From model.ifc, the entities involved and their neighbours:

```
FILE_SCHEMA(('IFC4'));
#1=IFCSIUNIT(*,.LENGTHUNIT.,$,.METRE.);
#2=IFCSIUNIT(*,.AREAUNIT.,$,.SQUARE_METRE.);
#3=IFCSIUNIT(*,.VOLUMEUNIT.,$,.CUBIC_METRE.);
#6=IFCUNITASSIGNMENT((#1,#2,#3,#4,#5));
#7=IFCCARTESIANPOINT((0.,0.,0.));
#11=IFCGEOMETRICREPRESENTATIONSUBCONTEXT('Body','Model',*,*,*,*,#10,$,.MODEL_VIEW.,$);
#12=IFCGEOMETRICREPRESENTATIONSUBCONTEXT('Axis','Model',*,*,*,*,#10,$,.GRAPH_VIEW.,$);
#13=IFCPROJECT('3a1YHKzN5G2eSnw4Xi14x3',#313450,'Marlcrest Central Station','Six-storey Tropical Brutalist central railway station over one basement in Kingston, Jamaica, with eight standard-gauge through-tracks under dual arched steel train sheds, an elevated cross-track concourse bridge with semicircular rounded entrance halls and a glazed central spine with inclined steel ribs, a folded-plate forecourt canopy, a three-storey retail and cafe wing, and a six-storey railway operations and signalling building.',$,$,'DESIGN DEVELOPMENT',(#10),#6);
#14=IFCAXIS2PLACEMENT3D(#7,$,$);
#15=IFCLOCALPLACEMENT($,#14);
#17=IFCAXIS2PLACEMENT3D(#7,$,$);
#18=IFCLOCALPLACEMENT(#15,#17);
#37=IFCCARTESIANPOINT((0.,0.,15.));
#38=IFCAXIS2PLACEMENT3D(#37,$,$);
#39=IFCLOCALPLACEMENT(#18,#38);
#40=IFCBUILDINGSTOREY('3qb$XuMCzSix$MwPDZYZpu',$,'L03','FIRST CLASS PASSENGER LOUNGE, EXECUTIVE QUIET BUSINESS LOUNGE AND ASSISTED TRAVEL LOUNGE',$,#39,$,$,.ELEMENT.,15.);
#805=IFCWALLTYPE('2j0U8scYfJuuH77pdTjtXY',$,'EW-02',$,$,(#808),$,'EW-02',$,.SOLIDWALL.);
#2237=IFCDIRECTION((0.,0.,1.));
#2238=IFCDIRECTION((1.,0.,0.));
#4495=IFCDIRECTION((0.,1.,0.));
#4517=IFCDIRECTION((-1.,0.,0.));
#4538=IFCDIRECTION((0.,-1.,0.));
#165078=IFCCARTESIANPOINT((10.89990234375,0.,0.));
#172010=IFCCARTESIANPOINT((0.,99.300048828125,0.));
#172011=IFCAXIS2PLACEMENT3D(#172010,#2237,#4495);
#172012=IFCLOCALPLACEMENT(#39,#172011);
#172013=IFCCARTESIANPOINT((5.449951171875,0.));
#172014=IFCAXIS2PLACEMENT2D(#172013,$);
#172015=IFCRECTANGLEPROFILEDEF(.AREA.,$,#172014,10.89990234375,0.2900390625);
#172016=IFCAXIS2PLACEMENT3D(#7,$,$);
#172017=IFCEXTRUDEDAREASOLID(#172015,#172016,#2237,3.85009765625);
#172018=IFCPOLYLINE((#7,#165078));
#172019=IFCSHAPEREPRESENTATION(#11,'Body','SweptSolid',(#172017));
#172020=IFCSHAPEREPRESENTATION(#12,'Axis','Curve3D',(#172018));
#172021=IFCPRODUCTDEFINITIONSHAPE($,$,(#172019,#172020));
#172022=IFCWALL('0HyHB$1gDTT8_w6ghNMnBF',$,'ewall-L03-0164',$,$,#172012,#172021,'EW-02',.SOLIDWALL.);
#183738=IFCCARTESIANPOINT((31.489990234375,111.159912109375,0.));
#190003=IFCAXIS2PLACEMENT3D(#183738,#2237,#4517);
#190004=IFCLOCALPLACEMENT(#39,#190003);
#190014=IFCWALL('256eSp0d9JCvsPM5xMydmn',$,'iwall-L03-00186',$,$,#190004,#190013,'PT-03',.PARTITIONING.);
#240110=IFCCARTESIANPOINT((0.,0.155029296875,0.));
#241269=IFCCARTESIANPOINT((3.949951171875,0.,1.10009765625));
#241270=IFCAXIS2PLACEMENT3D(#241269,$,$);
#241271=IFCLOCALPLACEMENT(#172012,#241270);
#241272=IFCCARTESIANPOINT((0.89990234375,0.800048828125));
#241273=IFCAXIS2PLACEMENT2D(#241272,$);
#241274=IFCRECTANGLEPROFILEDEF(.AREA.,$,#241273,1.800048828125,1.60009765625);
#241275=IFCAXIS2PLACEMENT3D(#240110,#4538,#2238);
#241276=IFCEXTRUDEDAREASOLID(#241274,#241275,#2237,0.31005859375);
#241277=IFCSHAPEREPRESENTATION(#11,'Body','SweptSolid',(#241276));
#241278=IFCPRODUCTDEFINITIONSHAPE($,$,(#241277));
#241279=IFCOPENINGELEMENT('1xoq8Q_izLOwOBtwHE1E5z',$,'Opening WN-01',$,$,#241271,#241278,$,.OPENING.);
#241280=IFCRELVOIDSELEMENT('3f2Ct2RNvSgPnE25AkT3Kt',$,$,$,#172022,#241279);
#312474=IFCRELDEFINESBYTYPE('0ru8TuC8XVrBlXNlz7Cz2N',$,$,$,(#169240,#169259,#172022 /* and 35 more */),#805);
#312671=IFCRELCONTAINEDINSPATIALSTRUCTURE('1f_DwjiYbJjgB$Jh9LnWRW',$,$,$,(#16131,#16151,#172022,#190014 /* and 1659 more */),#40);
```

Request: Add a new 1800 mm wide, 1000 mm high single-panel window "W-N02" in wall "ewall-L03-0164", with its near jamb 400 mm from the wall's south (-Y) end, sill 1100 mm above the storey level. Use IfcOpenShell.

```python
import numpy as np
import ifcopenshell
import ifcopenshell.api.feature
import ifcopenshell.api.geometry
import ifcopenshell.api.root
import ifcopenshell.api.spatial
import ifcopenshell.geom
import ifcopenshell.util.element
import ifcopenshell.util.placement
import ifcopenshell.util.representation
import ifcopenshell.util.shape
import ifcopenshell.util.unit

model = ifcopenshell.open("model.ifc")
unit_scale = ifcopenshell.util.unit.calculate_unit_scale(model)
settings = ifcopenshell.geom.settings()


def volume(element):
    """Net volume in cubic metres, openings subtracted."""
    shape = ifcopenshell.geom.create_shape(settings, element)
    return ifcopenshell.util.shape.get_volume(shape.geometry)


wall = model.by_guid("0HyHB$1gDTT8_w6ghNMnBF")
storey = ifcopenshell.util.element.get_container(wall, ifc_class="IfcBuildingStorey")
context = ifcopenshell.util.representation.get_context(model, "Model", "Body", "MODEL_VIEW")
before = volume(wall)

width, height, from_end, sill = 1.8, 1, 0.4, 1.1  # metres

# The wall runs along its own X axis, and the end named is its -X end.
wall_shape = ifcopenshell.geom.create_shape(settings, wall)
x, y, z = ifcopenshell.util.shape.get_vertices(wall_shape.geometry).T
start = x.min() + from_end
face, thickness = float(y.min()), float(y.max() - y.min())
wall_matrix = ifcopenshell.util.placement.get_local_placement(wall.ObjectPlacement)
level = ifcopenshell.util.placement.get_local_placement(storey.ObjectPlacement)[2, 3]


def in_wall(x, y):
    """Placement at x, y metres in the wall's axes, at sill height."""
    matrix = wall_matrix.copy()
    matrix[:, 3] = wall_matrix @ np.array([x / unit_scale, y / unit_scale, 0.0, 1.0])
    matrix[2, 3] = level + sill / unit_scale
    return matrix


# Opening: a box that overshoots both wall faces by 50 mm.
opening = ifcopenshell.api.root.create_entity(model, ifc_class="IfcOpeningElement", predefined_type="OPENING")
box = ifcopenshell.api.geometry.add_wall_representation(
    model, context=context, length=width, height=height, thickness=thickness + 0.1
)
ifcopenshell.api.geometry.assign_representation(model, product=opening, representation=box)
ifcopenshell.api.geometry.edit_object_placement(model, product=opening, matrix=in_wall(start, face - 0.05), is_si=False)
ifcopenshell.api.feature.add_feature(model, feature=opening, element=wall)

window = ifcopenshell.api.root.create_entity(model, ifc_class="IfcWindow", name="W-N02", predefined_type="WINDOW")
window.OverallWidth, window.OverallHeight = width / unit_scale, height / unit_scale
window.PartitioningType = "SINGLE_PANEL"
body = ifcopenshell.api.geometry.add_window_representation(
    model,
    context=context,
    overall_width=window.OverallWidth,
    overall_height=window.OverallHeight,
    partition_type="SINGLE_PANEL",
)
ifcopenshell.api.geometry.assign_representation(model, product=window, representation=body)
ifcopenshell.api.spatial.assign_container(model, products=[window], relating_structure=storey)
ifcopenshell.api.feature.add_filling(model, opening=opening, element=window)

# Centre the window in the wall's thickness.
ifcopenshell.api.geometry.edit_object_placement(model, product=window, matrix=in_wall(start, face), is_si=False)
window_shape = ifcopenshell.geom.create_shape(settings, window)
depth = ifcopenshell.util.shape.get_vertices(window_shape.geometry)[:, 1]
offset = face + thickness / 2 - (depth.min() + depth.max()) / 2
ifcopenshell.api.geometry.edit_object_placement(model, product=window, matrix=in_wall(start, offset), is_si=False)

after = volume(wall)

print(f"wall volume {before:.3f} -> {after:.3f} m3")

model.write("model_edited.ifc")
```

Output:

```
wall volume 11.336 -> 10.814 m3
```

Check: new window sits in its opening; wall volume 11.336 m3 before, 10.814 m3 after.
